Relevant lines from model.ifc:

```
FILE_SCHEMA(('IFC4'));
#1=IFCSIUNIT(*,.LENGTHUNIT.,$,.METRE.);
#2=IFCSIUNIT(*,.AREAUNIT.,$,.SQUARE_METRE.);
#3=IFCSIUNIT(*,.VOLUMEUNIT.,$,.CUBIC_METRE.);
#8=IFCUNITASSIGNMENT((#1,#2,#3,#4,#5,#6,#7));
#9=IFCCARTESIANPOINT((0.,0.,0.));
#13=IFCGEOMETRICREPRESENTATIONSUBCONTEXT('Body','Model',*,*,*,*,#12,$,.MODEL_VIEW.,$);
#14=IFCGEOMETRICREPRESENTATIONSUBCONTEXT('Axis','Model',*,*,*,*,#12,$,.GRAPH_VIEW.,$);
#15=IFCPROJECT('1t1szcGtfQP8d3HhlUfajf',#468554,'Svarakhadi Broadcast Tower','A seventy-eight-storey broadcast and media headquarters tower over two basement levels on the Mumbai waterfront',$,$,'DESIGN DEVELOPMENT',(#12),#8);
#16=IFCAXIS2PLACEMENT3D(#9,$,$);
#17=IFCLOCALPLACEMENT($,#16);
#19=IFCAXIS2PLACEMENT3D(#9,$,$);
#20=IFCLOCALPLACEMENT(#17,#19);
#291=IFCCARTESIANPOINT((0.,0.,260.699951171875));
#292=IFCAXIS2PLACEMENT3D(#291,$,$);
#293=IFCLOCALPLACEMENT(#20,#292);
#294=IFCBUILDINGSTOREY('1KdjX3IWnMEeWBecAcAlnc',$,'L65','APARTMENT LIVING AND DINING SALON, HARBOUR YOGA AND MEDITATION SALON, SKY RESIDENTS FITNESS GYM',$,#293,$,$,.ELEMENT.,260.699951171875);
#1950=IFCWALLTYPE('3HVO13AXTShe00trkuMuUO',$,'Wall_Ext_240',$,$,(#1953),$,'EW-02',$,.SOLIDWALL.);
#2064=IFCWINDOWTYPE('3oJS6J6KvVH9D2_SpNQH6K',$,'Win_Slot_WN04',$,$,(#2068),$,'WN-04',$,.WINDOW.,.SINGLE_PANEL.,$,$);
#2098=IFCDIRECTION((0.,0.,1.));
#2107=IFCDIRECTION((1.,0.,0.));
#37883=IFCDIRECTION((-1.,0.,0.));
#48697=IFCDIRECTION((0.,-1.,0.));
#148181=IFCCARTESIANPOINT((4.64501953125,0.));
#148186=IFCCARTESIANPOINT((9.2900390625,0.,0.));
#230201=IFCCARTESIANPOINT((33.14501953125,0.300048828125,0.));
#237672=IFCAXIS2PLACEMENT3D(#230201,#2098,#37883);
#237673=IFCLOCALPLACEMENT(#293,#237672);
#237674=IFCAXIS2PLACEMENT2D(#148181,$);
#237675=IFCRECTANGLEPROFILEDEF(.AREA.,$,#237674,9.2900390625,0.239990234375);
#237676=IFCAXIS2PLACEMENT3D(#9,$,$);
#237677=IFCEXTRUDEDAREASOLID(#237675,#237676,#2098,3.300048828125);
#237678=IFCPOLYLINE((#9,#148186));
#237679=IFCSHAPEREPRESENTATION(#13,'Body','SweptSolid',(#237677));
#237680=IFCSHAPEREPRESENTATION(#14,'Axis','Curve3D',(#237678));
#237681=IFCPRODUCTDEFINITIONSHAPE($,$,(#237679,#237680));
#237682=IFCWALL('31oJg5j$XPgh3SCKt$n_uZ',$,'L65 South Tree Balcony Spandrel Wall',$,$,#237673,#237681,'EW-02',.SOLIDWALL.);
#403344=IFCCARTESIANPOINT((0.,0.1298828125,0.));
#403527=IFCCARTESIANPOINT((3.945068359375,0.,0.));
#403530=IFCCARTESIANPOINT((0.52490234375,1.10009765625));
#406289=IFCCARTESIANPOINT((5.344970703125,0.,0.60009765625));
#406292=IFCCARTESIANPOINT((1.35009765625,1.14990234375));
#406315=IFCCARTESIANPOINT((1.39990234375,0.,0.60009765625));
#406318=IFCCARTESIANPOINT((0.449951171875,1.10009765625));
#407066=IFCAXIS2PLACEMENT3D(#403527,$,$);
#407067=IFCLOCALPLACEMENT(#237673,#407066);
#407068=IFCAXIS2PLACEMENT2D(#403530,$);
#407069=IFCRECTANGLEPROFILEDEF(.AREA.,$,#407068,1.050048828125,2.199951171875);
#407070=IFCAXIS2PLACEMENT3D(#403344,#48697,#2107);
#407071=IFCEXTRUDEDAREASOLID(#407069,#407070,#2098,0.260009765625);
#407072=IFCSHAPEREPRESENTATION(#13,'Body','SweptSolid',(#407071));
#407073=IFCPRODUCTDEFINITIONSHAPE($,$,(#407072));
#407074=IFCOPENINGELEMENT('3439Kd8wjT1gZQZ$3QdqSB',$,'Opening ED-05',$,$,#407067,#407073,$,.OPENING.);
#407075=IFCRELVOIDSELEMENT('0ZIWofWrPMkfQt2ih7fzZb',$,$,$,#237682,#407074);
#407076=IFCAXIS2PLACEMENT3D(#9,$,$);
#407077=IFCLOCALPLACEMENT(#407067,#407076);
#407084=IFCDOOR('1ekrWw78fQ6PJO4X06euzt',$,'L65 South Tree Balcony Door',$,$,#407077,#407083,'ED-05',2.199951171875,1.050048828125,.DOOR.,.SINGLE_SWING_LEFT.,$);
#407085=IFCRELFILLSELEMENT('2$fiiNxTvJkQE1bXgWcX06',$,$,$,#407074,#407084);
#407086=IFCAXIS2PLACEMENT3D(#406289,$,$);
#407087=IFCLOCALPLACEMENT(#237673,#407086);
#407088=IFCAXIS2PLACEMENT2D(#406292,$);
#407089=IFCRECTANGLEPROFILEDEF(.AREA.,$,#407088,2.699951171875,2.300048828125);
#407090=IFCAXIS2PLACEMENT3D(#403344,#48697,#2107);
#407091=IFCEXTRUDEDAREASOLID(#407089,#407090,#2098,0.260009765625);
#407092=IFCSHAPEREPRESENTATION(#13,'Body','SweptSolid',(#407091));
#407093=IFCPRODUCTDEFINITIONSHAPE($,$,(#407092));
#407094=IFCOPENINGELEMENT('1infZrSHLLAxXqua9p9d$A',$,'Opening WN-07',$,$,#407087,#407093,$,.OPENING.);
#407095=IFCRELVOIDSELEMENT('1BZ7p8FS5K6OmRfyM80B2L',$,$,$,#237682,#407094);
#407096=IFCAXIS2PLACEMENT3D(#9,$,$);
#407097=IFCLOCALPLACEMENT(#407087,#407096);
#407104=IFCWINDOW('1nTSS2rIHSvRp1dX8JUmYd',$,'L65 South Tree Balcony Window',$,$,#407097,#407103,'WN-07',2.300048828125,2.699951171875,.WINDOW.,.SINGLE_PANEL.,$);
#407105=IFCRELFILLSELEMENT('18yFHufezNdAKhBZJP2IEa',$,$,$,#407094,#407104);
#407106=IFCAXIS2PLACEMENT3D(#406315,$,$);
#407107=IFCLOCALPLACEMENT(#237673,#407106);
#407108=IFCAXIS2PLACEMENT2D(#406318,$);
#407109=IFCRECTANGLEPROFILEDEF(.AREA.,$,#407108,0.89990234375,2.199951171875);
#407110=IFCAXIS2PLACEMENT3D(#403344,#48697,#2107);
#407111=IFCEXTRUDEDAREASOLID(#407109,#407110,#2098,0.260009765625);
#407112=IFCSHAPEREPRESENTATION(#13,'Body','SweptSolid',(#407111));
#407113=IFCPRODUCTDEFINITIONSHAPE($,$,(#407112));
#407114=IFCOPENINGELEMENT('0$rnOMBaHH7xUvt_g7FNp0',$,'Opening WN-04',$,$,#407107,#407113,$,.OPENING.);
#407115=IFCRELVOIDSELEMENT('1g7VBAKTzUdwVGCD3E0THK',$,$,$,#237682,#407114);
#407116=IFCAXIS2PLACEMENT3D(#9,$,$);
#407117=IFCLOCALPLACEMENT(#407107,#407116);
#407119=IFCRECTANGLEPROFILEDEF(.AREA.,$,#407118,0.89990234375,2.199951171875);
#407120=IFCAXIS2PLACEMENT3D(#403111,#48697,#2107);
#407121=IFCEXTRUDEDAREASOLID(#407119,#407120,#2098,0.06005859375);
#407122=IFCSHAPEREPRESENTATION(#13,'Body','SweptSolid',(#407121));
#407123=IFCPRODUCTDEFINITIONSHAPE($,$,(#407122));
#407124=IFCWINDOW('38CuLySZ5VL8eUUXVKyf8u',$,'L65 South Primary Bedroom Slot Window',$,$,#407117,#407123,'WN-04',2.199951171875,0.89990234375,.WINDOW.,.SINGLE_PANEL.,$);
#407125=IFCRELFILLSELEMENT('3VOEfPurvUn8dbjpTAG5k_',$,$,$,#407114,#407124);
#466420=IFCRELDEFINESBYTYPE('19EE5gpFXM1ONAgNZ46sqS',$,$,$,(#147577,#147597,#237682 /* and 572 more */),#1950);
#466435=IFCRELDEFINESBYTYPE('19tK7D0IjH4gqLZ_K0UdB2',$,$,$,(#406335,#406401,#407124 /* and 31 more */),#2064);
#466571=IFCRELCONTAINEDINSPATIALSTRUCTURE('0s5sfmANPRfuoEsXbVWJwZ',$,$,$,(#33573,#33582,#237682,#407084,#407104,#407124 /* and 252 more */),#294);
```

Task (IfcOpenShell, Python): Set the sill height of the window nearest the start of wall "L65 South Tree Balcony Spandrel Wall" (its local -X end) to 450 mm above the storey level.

```python
import numpy as np
import ifcopenshell
import ifcopenshell.api.geometry
import ifcopenshell.geom
import ifcopenshell.util.element
import ifcopenshell.util.placement
import ifcopenshell.util.shape
import ifcopenshell.util.unit

model = ifcopenshell.open("model.ifc")
unit_scale = ifcopenshell.util.unit.calculate_unit_scale(model)

window = model.by_guid("38CuLySZ5VL8eUUXVKyf8u")
opening = window.FillsVoids[0].RelatingOpeningElement
storey = ifcopenshell.util.element.get_container(window, ifc_class="IfcBuildingStorey")
level = ifcopenshell.util.placement.get_local_placement(storey.ObjectPlacement)[2, 3]

# The opening's origin need not be at the sill, so measure its lowest point.
shape = ifcopenshell.geom.create_shape(ifcopenshell.geom.settings(), opening)
bottom = ifcopenshell.util.shape.get_shape_bottom_elevation(shape, shape.geometry) / unit_scale
dz = level + 0.45 / unit_scale - bottom

shift = np.array([0.0, 0.0, dz])
# The window is placed relative to its opening, so it follows when the opening moves.
matrix = ifcopenshell.util.placement.get_local_placement(opening.ObjectPlacement)
matrix[:3, 3] += shift
ifcopenshell.api.geometry.edit_object_placement(
    model, product=opening, matrix=matrix, is_si=False, should_transform_children=True
)

print(f"moved by {dz * unit_scale:+.3f} m")

model.write("model_edited.ifc")
```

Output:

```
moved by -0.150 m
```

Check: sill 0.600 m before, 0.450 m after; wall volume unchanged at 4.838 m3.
